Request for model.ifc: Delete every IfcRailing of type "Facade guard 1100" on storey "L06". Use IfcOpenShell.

First a look at what the model holds.

```python
import ifcopenshell
import ifcopenshell.util.element

model = ifcopenshell.open("model.ifc")
print(model.schema)
storey = next(s for s in model.by_type("IfcBuildingStorey") if s.Name == "L06")
railings = [e for e in ifcopenshell.util.element.get_decomposition(storey) if e.is_a("IfcRailing")]
seen = {}
for e in railings:
    element_type = ifcopenshell.util.element.get_type(e)
    name = element_type.Name if element_type not in (None, e) else None
    seen[name] = seen.get(name, 0) + 1
for name, count in sorted(seen.items(), key=str):
    print(count, "x", name)
```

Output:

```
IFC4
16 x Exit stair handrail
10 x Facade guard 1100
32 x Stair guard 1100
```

```python
import ifcopenshell
import ifcopenshell.api.root
import ifcopenshell.util.element

model = ifcopenshell.open("model.ifc")

storey = next(s for s in model.by_type("IfcBuildingStorey") if s.Name == "L06")
railings = [e for e in ifcopenshell.util.element.get_decomposition(storey) if e.is_a("IfcRailing")]
targets = [e for e in railings if (t := ifcopenshell.util.element.get_type(e)) not in (None, e) and t.Name == "Facade guard 1100"]

for e in targets:
    ifcopenshell.api.root.remove_product(model, product=e)
print(len(targets), "removed")

model.write("model_rev.ifc")
```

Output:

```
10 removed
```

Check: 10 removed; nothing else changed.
